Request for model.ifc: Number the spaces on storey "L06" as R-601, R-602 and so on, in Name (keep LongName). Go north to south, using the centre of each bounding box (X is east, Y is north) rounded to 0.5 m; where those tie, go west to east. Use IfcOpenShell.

First a look at what the model holds.

```python
import ifcopenshell
import ifcopenshell.util.element
import ifcopenshell.util.placement

model = ifcopenshell.open("model.ifc")
print(model.schema)
storey = next(s for s in model.by_type("IfcBuildingStorey") if s.Name == "L06")
spaces = [e for e in ifcopenshell.util.element.get_decomposition(storey) if e.is_a("IfcSpace")]
for e in sorted(spaces, key=lambda e: e.id()):
    origin = ifcopenshell.util.placement.get_local_placement(e.ObjectPlacement)[:3, 3]
    print(e.id(), e.Name, e.LongName, origin.round(2) + 0.0, sep=" | ")
```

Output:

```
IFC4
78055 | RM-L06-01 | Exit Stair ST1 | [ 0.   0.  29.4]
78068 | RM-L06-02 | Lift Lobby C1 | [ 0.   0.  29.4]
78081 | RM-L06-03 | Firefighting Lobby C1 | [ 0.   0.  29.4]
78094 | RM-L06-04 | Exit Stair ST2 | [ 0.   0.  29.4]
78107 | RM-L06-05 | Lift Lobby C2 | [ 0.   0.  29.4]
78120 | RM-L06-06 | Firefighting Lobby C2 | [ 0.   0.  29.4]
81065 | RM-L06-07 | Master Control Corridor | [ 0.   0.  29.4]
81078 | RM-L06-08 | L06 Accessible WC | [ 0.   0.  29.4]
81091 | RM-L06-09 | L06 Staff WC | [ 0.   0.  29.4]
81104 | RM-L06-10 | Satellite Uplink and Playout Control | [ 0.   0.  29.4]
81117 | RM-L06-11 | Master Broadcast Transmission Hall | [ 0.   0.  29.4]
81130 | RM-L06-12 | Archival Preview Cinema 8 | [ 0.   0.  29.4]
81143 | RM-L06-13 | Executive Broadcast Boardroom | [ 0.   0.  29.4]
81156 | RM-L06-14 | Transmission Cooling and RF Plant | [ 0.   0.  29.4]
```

```python
import ifcopenshell
import ifcopenshell.geom
import ifcopenshell.util.element
import ifcopenshell.util.shape

model = ifcopenshell.open("model.ifc")
settings = ifcopenshell.geom.settings()
settings.set("use-world-coords", True)


def centre(element):
    shape = ifcopenshell.geom.create_shape(settings, element)
    return ifcopenshell.util.shape.get_bbox_centroid(shape.geometry)


storey = next(s for s in model.by_type("IfcBuildingStorey") if s.Name == "L06")
spaces = [e for e in ifcopenshell.util.element.get_decomposition(storey) if e.is_a("IfcSpace")]

# Insertion points can sit at a corner or the storey origin, so sort by the geometry (in metres).
centres = {e: centre(e) for e in spaces}
spaces.sort(key=lambda e: (-round(centres[e][1] / 0.5), centres[e][0]))

for i, e in enumerate(spaces, start=1):
    number = f"R-6{i:02d}"
    e.Name = number
    print(e.id(), number)

model.write("model-out.ifc")
```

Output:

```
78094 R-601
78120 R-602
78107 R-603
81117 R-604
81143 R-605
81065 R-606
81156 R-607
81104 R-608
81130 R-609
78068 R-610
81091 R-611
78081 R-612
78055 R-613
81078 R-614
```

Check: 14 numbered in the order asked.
